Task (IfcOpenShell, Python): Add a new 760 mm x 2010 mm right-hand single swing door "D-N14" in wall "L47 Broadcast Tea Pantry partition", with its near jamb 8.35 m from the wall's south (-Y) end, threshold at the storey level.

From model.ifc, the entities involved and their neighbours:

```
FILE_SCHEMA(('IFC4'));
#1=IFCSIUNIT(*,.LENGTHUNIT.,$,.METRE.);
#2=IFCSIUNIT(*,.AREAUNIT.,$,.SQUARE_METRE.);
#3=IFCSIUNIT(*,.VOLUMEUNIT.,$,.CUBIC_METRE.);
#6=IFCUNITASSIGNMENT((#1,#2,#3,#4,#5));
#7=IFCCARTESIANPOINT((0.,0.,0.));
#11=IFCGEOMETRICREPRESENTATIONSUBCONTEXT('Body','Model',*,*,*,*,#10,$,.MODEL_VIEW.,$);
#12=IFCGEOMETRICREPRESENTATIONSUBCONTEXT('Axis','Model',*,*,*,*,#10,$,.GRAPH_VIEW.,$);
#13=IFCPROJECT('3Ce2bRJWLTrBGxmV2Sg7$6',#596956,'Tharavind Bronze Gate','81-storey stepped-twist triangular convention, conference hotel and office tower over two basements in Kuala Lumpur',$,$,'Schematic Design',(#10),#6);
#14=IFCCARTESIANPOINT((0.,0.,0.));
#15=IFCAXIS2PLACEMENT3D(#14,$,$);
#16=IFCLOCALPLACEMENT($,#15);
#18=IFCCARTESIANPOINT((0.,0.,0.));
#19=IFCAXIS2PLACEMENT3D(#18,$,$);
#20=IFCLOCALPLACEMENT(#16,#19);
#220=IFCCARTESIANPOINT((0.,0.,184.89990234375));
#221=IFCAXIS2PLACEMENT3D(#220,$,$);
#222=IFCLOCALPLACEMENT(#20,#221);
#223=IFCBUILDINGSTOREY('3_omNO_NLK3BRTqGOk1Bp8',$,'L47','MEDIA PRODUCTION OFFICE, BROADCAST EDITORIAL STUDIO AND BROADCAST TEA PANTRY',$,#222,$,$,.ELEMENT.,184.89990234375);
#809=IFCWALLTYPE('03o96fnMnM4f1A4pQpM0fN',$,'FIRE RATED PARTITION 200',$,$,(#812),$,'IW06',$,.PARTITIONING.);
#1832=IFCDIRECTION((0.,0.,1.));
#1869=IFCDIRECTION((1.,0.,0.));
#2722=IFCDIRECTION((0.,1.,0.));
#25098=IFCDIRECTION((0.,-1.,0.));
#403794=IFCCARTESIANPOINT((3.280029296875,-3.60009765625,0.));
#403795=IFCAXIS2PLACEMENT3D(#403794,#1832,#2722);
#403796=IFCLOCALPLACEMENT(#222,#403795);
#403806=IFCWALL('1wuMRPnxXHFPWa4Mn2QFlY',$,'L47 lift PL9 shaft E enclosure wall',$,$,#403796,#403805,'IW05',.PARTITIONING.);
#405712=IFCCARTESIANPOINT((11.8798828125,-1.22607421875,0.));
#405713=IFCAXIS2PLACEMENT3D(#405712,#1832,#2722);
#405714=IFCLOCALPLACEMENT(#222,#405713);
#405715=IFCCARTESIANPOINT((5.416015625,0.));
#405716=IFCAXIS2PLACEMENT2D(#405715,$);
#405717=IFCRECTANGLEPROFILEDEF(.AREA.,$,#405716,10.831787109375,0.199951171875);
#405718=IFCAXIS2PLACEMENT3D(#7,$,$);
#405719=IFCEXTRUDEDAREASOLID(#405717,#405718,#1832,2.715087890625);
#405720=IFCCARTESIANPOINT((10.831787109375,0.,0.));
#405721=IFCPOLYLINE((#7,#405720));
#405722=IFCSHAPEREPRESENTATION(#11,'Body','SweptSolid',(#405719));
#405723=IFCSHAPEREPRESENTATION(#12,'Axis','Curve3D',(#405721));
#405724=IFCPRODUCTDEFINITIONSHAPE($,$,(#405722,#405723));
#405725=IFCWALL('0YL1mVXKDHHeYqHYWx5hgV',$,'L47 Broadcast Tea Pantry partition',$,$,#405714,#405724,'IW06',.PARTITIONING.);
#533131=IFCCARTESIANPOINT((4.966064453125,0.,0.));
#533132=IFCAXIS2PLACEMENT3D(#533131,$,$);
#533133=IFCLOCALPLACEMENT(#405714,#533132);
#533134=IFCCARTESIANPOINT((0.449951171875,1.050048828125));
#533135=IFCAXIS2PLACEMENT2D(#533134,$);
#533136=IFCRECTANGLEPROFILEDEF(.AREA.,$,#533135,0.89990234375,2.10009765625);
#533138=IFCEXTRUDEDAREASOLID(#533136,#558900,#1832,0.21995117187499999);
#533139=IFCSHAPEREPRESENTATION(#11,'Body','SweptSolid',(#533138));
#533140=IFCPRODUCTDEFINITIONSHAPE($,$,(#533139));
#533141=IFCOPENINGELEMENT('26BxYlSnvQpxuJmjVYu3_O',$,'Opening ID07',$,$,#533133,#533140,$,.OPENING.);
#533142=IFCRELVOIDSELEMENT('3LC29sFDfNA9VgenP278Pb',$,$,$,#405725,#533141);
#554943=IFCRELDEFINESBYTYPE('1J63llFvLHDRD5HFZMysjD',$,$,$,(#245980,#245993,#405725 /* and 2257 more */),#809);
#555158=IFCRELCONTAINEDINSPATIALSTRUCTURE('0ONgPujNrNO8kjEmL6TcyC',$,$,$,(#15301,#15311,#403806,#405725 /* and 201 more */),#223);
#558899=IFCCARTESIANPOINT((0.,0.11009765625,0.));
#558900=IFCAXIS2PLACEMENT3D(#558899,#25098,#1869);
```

```python
import numpy as np
import ifcopenshell
import ifcopenshell.api.feature
import ifcopenshell.api.geometry
import ifcopenshell.api.root
import ifcopenshell.api.spatial
import ifcopenshell.geom
import ifcopenshell.util.element
import ifcopenshell.util.placement
import ifcopenshell.util.representation
import ifcopenshell.util.shape
import ifcopenshell.util.unit

model = ifcopenshell.open("model.ifc")
unit_scale = ifcopenshell.util.unit.calculate_unit_scale(model)
settings = ifcopenshell.geom.settings()


def volume(element):
    """Net volume in cubic metres, openings subtracted."""
    shape = ifcopenshell.geom.create_shape(settings, element)
    return ifcopenshell.util.shape.get_volume(shape.geometry)


wall = model.by_guid("0YL1mVXKDHHeYqHYWx5hgV")
storey = ifcopenshell.util.element.get_container(wall, ifc_class="IfcBuildingStorey")
context = ifcopenshell.util.representation.get_context(model, "Model", "Body", "MODEL_VIEW")
before = volume(wall)

width, height, from_end, sill = 0.76, 2.01, 8.35, 0.0  # metres

# The wall runs along its own X axis, and the end named is its -X end.
wall_shape = ifcopenshell.geom.create_shape(settings, wall)
x, y, z = ifcopenshell.util.shape.get_vertices(wall_shape.geometry).T
start = x.min() + from_end
face, thickness = float(y.min()), float(y.max() - y.min())
wall_matrix = ifcopenshell.util.placement.get_local_placement(wall.ObjectPlacement)
level = ifcopenshell.util.placement.get_local_placement(storey.ObjectPlacement)[2, 3]


def in_wall(x, y):
    """Placement at x, y metres in the wall's axes, at sill height."""
    matrix = wall_matrix.copy()
    matrix[:, 3] = wall_matrix @ np.array([x / unit_scale, y / unit_scale, 0.0, 1.0])
    matrix[2, 3] = level + sill / unit_scale
    return matrix


# Opening: a box that overshoots both wall faces by 50 mm.
opening = ifcopenshell.api.root.create_entity(model, ifc_class="IfcOpeningElement", predefined_type="OPENING")
box = ifcopenshell.api.geometry.add_wall_representation(
    model, context=context, length=width, height=height, thickness=thickness + 0.1
)
ifcopenshell.api.geometry.assign_representation(model, product=opening, representation=box)
ifcopenshell.api.geometry.edit_object_placement(model, product=opening, matrix=in_wall(start, face - 0.05), is_si=False)
ifcopenshell.api.feature.add_feature(model, feature=opening, element=wall)

door = ifcopenshell.api.root.create_entity(model, ifc_class="IfcDoor", name="D-N14", predefined_type="DOOR")
door.OverallWidth, door.OverallHeight = width / unit_scale, height / unit_scale
door.OperationType = "SINGLE_SWING_RIGHT"
body = ifcopenshell.api.geometry.add_door_representation(
    model,
    context=context,
    overall_width=door.OverallWidth,
    overall_height=door.OverallHeight,
    operation_type="SINGLE_SWING_RIGHT",
    lining_properties={"LiningDepth": thickness / unit_scale, "ThresholdDepth": thickness / unit_scale},
)
ifcopenshell.api.geometry.assign_representation(model, product=door, representation=body)
ifcopenshell.api.spatial.assign_container(model, products=[door], relating_structure=storey)
ifcopenshell.api.feature.add_filling(model, opening=opening, element=door)

# The lining spans the wall, so the door starts at the wall face.
ifcopenshell.api.geometry.edit_object_placement(model, product=door, matrix=in_wall(start, face), is_si=False)

after = volume(wall)

print(f"wall volume {before:.3f} -> {after:.3f} m3")

model.write("model_v2.ifc")
```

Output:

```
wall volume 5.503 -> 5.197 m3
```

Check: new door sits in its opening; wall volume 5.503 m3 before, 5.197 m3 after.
